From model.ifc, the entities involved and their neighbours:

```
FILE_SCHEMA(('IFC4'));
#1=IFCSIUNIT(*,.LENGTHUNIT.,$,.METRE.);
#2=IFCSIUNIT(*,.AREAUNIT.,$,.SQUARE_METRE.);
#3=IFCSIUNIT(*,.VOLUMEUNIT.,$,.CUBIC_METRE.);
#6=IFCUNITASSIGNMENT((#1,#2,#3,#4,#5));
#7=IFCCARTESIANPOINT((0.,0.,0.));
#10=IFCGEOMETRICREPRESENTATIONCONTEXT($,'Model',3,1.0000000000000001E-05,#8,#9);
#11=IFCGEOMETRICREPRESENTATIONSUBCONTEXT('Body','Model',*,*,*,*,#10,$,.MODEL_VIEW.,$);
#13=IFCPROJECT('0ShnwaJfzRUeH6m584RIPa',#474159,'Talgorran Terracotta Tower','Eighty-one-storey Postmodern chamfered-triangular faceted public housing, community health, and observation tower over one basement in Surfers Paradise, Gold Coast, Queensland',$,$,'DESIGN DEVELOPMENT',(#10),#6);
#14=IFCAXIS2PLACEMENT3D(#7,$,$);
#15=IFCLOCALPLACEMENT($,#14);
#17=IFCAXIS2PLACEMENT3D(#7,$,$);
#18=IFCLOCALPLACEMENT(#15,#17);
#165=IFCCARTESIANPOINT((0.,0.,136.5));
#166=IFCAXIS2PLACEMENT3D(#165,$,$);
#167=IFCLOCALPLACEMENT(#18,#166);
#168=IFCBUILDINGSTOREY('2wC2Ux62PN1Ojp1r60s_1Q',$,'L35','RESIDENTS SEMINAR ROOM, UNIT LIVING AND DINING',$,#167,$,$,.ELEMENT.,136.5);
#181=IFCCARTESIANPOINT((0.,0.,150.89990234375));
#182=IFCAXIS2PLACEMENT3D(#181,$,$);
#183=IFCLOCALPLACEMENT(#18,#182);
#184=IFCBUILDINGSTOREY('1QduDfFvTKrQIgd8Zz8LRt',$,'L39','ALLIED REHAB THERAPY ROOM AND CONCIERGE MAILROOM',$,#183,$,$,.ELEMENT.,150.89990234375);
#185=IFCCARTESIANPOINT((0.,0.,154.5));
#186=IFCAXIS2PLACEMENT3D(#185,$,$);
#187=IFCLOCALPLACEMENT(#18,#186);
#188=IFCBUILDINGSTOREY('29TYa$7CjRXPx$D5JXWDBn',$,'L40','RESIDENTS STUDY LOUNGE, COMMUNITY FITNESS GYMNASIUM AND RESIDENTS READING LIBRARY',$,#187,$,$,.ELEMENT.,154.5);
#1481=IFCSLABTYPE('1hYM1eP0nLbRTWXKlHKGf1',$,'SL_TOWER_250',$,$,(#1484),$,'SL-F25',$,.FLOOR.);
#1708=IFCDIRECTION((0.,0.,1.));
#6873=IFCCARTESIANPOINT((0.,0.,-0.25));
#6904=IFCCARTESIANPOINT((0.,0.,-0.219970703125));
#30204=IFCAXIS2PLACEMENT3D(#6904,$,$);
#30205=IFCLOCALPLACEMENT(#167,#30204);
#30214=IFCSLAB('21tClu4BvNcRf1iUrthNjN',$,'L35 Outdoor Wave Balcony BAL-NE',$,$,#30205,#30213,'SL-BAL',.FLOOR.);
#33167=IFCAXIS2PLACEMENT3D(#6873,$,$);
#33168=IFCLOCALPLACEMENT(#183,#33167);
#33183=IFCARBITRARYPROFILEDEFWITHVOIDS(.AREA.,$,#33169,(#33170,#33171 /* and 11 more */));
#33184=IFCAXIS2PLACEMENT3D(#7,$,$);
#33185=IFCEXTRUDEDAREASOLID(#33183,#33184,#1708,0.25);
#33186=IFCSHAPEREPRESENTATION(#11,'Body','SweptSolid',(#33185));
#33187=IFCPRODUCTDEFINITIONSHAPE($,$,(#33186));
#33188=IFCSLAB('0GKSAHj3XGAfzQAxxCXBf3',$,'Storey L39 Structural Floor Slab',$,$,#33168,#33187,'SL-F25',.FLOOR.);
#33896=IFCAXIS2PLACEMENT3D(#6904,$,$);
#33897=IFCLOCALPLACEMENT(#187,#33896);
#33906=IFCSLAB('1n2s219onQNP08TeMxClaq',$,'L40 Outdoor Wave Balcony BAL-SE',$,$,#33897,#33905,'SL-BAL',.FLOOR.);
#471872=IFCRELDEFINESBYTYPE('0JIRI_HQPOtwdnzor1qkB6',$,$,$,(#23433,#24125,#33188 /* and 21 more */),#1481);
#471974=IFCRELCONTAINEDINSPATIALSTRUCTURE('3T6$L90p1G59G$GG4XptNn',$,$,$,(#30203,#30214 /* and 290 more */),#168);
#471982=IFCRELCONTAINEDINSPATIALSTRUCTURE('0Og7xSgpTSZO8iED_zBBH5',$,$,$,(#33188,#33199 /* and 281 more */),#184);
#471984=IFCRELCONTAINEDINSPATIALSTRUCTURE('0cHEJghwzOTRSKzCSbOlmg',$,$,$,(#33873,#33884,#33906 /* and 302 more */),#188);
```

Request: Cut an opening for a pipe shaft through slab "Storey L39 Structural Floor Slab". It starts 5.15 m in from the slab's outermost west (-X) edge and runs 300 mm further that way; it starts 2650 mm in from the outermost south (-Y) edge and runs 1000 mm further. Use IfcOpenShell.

```python
import numpy as np
import ifcopenshell
import ifcopenshell.api.feature
import ifcopenshell.api.geometry
import ifcopenshell.api.root
import ifcopenshell.geom
import ifcopenshell.util.placement
import ifcopenshell.util.representation
import ifcopenshell.util.shape
import ifcopenshell.util.unit

model = ifcopenshell.open("model.ifc")
unit_scale = ifcopenshell.util.unit.calculate_unit_scale(model)
settings = ifcopenshell.geom.settings()


def volume(element):
    """Net volume in cubic metres, openings subtracted."""
    shape = ifcopenshell.geom.create_shape(settings, element)
    return ifcopenshell.util.shape.get_volume(shape.geometry)


slab = model.by_guid("0GKSAHj3XGAfzQAxxCXBf3")
before = volume(slab)

# Extent in the slab's own axes, in metres. The edges named are its -X and -Y sides.
slab_shape = ifcopenshell.geom.create_shape(settings, slab)
vertices = ifcopenshell.util.shape.get_vertices(slab_shape.geometry)
x_min, y_min, bottom = vertices.min(axis=0)
top = vertices[:, 2].max()

opening = ifcopenshell.api.root.create_entity(model, ifc_class="IfcOpeningElement", name="Pipe shaft opening", predefined_type="OPENING")
context = ifcopenshell.util.representation.get_context(model, "Model", "Body", "MODEL_VIEW")
width, depth = 0.3, 1
outline = [(0.0, 0.0), (width, 0.0), (width, depth), (0.0, depth), (0.0, 0.0)]
# Overshoot both faces by 50 mm so the cut is clean.
shape = ifcopenshell.api.geometry.add_slab_representation(
    model, context=context, depth=top - bottom + 0.1, polyline=outline
)
ifcopenshell.api.geometry.assign_representation(model, product=opening, representation=shape)

matrix = ifcopenshell.util.placement.get_local_placement(slab.ObjectPlacement)
matrix[:, 3] = matrix @ np.append(np.array([x_min + 5.15, y_min + 2.65, bottom - 0.05]) / unit_scale, 1.0)
ifcopenshell.api.geometry.edit_object_placement(model, product=opening, matrix=matrix, is_si=False)
ifcopenshell.api.feature.add_feature(model, feature=opening, element=slab)

after = volume(slab)

print(f"slab volume {before:.3f} -> {after:.3f} m3")

model.write("model_updated.ifc")
```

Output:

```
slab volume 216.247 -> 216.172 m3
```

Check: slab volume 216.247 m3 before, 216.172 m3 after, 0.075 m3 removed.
